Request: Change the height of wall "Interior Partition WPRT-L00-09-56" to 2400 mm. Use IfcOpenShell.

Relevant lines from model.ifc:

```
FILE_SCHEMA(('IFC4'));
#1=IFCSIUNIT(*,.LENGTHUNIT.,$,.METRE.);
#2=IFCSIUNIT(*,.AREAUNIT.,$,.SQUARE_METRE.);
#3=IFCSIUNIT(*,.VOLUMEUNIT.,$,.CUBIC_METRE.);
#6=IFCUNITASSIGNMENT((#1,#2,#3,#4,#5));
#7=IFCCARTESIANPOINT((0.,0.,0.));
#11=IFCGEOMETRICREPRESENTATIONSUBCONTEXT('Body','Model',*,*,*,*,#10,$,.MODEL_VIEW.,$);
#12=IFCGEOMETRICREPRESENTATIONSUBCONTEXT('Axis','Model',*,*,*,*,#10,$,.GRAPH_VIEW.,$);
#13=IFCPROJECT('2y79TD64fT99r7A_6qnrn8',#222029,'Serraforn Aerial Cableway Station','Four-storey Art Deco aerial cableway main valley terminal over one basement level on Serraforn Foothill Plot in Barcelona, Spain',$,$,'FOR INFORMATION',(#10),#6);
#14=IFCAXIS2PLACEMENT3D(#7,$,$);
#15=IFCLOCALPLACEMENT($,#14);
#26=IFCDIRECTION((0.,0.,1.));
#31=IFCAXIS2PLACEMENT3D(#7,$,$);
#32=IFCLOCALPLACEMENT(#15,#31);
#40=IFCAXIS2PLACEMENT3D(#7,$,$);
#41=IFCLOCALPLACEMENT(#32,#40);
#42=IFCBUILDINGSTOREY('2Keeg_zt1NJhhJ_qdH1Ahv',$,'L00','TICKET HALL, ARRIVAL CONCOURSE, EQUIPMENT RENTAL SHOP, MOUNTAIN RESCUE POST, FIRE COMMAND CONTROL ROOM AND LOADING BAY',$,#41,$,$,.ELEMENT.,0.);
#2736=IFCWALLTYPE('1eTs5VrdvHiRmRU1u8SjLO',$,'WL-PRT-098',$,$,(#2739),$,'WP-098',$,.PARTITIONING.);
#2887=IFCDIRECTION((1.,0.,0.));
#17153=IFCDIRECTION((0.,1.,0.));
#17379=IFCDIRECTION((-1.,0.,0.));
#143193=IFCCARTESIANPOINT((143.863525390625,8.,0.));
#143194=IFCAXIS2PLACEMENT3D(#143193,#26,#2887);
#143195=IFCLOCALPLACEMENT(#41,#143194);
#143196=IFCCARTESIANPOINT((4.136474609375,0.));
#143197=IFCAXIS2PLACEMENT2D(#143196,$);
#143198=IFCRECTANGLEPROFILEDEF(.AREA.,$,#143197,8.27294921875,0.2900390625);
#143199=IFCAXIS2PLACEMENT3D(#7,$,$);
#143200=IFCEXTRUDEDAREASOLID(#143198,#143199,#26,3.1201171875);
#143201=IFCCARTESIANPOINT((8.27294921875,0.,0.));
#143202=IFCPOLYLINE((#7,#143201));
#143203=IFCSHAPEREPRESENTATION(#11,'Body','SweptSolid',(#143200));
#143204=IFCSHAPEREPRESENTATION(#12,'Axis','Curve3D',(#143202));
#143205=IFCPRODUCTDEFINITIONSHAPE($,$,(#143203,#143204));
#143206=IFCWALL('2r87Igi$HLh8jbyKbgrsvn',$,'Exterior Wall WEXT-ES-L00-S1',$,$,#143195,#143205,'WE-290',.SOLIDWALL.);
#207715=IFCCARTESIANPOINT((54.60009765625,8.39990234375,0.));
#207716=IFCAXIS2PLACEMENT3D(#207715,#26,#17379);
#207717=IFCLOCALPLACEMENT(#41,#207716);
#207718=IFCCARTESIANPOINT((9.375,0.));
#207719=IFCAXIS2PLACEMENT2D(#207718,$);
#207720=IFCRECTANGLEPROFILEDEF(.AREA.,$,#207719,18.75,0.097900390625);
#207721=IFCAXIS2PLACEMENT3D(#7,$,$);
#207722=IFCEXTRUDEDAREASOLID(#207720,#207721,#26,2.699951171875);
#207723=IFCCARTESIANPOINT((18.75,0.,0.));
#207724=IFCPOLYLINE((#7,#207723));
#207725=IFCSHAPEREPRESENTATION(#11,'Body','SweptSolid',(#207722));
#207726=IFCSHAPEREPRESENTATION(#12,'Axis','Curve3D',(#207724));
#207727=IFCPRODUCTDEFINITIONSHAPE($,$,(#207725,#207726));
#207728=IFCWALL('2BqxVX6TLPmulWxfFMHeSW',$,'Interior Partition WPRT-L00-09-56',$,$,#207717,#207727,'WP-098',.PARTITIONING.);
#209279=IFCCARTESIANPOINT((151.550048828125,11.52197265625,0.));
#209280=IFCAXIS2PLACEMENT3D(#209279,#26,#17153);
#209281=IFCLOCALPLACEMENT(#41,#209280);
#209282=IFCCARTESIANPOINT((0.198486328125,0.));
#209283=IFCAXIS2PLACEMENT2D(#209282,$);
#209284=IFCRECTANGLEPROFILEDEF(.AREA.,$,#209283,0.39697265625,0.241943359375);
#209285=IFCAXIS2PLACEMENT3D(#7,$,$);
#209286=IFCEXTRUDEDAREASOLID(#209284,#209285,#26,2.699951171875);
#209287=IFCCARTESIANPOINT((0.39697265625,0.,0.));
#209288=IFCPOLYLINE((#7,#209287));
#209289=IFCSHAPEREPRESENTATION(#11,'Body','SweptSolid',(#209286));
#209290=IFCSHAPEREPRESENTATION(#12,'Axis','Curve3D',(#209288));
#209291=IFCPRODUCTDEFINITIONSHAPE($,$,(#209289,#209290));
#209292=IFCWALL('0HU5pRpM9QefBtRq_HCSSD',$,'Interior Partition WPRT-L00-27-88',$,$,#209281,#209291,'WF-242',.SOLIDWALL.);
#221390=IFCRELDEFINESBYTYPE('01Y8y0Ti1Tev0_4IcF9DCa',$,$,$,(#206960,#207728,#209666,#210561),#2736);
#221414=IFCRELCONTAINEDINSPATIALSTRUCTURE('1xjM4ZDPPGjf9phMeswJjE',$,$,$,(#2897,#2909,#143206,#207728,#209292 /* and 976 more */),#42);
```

```python
import ifcopenshell
import ifcopenshell.geom
import ifcopenshell.util.representation
import ifcopenshell.util.shape

model = ifcopenshell.open("model.ifc")
settings = ifcopenshell.geom.settings()


def volume(element):
    """Net volume in cubic metres, openings subtracted."""
    shape = ifcopenshell.geom.create_shape(settings, element)
    return ifcopenshell.util.shape.get_volume(shape.geometry)


wall = model.by_id(207728)
before = volume(wall)

body = ifcopenshell.util.representation.get_representation(wall, "Model", "Body")
solid = body.Items[0]
old_height = solid.Depth
solid.Depth = 2.4
after = volume(wall)

print(f"height {old_height:g} -> {solid.Depth:g}, volume {before:.3f} -> {after:.3f} m3")

model.write("model-out.ifc")
```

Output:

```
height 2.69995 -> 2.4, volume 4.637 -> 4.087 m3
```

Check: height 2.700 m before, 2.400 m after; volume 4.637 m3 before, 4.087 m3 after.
